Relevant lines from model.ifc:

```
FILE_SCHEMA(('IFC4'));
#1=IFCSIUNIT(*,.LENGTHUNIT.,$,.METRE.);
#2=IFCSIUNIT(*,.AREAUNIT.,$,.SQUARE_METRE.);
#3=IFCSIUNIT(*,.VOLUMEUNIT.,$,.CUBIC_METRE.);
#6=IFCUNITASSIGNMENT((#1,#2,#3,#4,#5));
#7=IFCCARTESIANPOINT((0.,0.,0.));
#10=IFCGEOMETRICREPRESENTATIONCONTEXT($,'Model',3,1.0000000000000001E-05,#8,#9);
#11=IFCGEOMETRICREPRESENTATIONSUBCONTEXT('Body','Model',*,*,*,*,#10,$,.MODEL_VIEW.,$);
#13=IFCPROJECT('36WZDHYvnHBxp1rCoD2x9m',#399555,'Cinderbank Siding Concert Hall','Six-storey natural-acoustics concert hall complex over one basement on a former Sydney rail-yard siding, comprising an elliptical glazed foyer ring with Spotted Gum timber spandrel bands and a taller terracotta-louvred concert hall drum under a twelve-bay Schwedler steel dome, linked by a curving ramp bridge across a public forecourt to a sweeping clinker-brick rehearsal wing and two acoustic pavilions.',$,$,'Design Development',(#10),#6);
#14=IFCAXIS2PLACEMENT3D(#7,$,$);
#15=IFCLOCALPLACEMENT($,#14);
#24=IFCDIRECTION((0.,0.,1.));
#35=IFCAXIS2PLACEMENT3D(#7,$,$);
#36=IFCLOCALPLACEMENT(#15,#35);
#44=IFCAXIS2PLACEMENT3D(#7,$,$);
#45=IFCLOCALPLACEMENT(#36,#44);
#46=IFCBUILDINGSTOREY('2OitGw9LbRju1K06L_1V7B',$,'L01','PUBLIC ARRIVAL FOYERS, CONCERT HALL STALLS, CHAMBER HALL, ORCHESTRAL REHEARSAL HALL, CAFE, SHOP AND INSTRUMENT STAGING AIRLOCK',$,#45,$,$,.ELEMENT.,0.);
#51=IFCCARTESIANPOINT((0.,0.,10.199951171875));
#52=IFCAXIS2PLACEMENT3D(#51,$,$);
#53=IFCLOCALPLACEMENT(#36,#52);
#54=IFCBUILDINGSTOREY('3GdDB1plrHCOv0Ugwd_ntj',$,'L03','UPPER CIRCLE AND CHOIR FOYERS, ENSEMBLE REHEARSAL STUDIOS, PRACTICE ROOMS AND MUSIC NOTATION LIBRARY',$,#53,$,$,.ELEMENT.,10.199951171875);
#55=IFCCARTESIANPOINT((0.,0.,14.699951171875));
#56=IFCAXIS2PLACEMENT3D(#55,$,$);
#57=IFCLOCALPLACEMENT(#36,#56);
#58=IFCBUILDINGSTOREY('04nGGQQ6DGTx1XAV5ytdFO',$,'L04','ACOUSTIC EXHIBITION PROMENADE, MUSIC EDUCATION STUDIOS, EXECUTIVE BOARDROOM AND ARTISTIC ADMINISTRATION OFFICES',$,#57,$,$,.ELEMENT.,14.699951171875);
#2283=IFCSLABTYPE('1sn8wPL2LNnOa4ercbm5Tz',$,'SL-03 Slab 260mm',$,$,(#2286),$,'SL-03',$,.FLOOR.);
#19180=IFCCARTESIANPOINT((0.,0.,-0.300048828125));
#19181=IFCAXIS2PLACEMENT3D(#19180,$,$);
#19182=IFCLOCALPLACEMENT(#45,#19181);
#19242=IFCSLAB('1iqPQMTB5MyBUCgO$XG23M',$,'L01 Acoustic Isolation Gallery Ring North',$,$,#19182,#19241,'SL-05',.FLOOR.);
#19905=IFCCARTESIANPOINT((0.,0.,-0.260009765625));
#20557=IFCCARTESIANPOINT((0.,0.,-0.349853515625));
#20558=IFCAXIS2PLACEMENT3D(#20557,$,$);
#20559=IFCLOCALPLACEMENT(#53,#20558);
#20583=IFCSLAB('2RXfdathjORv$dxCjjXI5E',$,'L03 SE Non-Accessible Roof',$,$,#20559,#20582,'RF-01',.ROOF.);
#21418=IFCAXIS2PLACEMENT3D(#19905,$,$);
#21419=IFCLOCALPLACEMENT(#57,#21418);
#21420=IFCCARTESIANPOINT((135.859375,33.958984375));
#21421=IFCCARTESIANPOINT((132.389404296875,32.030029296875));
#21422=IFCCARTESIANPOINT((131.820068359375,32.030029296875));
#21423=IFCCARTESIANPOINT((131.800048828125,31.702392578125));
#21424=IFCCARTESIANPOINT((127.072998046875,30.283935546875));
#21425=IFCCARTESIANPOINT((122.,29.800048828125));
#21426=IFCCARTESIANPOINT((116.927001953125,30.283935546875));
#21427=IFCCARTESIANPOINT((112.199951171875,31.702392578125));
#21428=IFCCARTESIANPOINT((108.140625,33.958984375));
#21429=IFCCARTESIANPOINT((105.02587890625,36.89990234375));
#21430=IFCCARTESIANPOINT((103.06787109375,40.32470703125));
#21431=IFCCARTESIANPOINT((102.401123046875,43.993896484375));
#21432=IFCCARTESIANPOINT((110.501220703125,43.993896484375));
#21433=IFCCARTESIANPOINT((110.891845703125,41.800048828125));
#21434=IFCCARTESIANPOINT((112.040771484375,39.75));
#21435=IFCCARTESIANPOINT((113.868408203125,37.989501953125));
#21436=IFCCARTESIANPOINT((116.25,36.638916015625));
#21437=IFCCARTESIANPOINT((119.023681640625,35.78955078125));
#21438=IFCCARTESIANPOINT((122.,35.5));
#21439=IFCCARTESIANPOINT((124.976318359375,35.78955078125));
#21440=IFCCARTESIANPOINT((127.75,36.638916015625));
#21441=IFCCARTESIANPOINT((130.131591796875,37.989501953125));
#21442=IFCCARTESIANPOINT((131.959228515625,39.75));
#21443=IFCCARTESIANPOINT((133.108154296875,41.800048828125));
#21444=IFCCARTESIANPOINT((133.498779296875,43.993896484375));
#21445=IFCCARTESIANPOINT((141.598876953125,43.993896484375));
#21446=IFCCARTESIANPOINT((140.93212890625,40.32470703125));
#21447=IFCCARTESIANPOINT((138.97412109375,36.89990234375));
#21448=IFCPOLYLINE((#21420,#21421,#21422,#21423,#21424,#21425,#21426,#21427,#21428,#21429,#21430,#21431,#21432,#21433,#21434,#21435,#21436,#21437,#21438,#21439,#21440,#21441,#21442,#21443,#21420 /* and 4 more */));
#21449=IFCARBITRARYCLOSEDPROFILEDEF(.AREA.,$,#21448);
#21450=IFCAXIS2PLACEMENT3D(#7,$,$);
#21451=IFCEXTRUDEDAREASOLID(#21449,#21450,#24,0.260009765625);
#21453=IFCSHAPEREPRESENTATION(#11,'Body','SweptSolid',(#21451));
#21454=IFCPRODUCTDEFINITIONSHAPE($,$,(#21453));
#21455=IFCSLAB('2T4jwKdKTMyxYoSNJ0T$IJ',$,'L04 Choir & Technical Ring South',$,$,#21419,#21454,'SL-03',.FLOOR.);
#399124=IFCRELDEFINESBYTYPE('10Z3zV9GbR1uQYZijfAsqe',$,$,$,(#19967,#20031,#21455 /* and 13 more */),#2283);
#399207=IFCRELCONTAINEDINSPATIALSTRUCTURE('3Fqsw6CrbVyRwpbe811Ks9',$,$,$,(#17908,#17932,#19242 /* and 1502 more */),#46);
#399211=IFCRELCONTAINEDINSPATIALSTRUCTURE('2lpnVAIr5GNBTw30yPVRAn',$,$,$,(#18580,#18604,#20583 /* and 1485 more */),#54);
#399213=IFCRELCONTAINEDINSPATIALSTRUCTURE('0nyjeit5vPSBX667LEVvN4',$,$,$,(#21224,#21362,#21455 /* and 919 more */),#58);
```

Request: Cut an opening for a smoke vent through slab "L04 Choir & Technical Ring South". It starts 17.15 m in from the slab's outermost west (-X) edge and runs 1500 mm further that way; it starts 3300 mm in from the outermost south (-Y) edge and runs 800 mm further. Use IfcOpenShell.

```python
import numpy as np
import ifcopenshell
import ifcopenshell.api.feature
import ifcopenshell.api.geometry
import ifcopenshell.api.root
import ifcopenshell.geom
import ifcopenshell.util.placement
import ifcopenshell.util.representation
import ifcopenshell.util.shape
import ifcopenshell.util.unit

model = ifcopenshell.open("model.ifc")
unit_scale = ifcopenshell.util.unit.calculate_unit_scale(model)
settings = ifcopenshell.geom.settings()


def volume(element):
    """Net volume in cubic metres, openings subtracted."""
    shape = ifcopenshell.geom.create_shape(settings, element)
    return ifcopenshell.util.shape.get_volume(shape.geometry)


slab = model.by_guid("2T4jwKdKTMyxYoSNJ0T$IJ")
before = volume(slab)

# Extent in the slab's own axes, in metres. The edges named are its -X and -Y sides.
slab_shape = ifcopenshell.geom.create_shape(settings, slab)
vertices = ifcopenshell.util.shape.get_vertices(slab_shape.geometry)
x_min, y_min, bottom = vertices.min(axis=0)
top = vertices[:, 2].max()

opening = ifcopenshell.api.root.create_entity(model, ifc_class="IfcOpeningElement", name="Smoke vent opening", predefined_type="OPENING")
context = ifcopenshell.util.representation.get_context(model, "Model", "Body", "MODEL_VIEW")
width, depth = 1.5, 0.8
outline = [(0.0, 0.0), (width, 0.0), (width, depth), (0.0, depth), (0.0, 0.0)]
# Overshoot both faces by 50 mm so the cut is clean.
shape = ifcopenshell.api.geometry.add_slab_representation(
    model, context=context, depth=top - bottom + 0.1, polyline=outline
)
ifcopenshell.api.geometry.assign_representation(model, product=opening, representation=shape)

matrix = ifcopenshell.util.placement.get_local_placement(slab.ObjectPlacement)
matrix[:, 3] = matrix @ np.append(np.array([x_min + 17.15, y_min + 3.3, bottom - 0.05]) / unit_scale, 1.0)
ifcopenshell.api.geometry.edit_object_placement(model, product=opening, matrix=matrix, is_si=False)
ifcopenshell.api.feature.add_feature(model, feature=opening, element=slab)

after = volume(slab)

print(f"slab volume {before:.3f} -> {after:.3f} m3")

model.write("model_edited.ifc")
```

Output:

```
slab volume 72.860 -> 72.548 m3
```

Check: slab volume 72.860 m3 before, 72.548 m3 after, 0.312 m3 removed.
